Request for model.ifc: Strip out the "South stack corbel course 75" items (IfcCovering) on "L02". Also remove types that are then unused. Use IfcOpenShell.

First a look at what the model holds.

```python
import ifcopenshell
import ifcopenshell.util.element

model = ifcopenshell.open("model.ifc")
print(model.schema)
storey = next(s for s in model.by_type("IfcBuildingStorey") if s.Name == "L02")
coverings = [e for e in ifcopenshell.util.element.get_decomposition(storey) if e.is_a("IfcCovering")]
seen = {}
for e in coverings:
    element_type = ifcopenshell.util.element.get_type(e)
    name = element_type.Name if element_type not in (None, e) else None
    seen[name] = seen.get(name, 0) + 1
for name, count in sorted(seen.items(), key=str):
    print(count, "x", name)
```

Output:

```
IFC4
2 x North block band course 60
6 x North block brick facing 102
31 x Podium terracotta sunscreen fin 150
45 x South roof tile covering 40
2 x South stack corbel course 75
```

```python
import ifcopenshell
import ifcopenshell.api.root
import ifcopenshell.util.element

model = ifcopenshell.open("model.ifc")

storey = next(s for s in model.by_type("IfcBuildingStorey") if s.Name == "L02")
coverings = [e for e in ifcopenshell.util.element.get_decomposition(storey) if e.is_a("IfcCovering")]
targets = [e for e in coverings if (t := ifcopenshell.util.element.get_type(e)) not in (None, e) and t.Name == "South stack corbel course 75"]
types = {ifcopenshell.util.element.get_type(e) for e in targets} - {None, *targets}

for e in targets:
    ifcopenshell.api.root.remove_product(model, product=e)
print(len(targets), "removed")

unused = [t for t in types if not ifcopenshell.util.element.get_types(t)]
for t in unused:
    ifcopenshell.api.root.remove_product(model, product=t)
print(len(unused), "unused types removed")

model.write("model_edited.ifc")
```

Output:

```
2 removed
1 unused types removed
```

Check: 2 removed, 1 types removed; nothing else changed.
